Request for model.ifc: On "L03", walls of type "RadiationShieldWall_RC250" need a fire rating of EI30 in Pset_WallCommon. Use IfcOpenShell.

First a look at what the model holds.

```python
import ifcopenshell
import ifcopenshell.util.element

model = ifcopenshell.open("model.ifc")
print(model.schema)
storey = next(s for s in model.by_type("IfcBuildingStorey") if s.Name == "L03")
walls = [e for e in ifcopenshell.util.element.get_decomposition(storey) if e.is_a("IfcWall")]
seen = {}
for e in walls:
    element_type = ifcopenshell.util.element.get_type(e)
    key = (element_type.Name if element_type != e and element_type else None, ifcopenshell.util.element.get_pset(e, "Pset_WallCommon", "FireRating"))
    seen[key] = seen.get(key, 0) + 1
for (name, value), count in sorted(seen.items(), key=str):
    print(count, "x", name, "|", value)
```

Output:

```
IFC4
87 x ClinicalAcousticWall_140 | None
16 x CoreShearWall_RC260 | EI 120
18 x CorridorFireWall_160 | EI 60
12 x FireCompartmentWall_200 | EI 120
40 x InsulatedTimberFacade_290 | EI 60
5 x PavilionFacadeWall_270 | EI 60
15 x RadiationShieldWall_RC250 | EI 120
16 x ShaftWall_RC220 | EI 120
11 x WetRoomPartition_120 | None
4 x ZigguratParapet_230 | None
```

```python
import ifcopenshell
import ifcopenshell.api.pset
import ifcopenshell.util.element

model = ifcopenshell.open("model.ifc")

storey = next(s for s in model.by_type("IfcBuildingStorey") if s.Name == "L03")
walls = [e for e in ifcopenshell.util.element.get_decomposition(storey) if e.is_a("IfcWall")]

count = 0
for e in walls:
    element_type = ifcopenshell.util.element.get_type(e)
    if element_type in (None, e) or element_type.Name != "RadiationShieldWall_RC250":
        continue
    # add_pset returns the element's existing set when there is one.
    pset = ifcopenshell.api.pset.add_pset(model, product=e, name="Pset_WallCommon")
    ifcopenshell.api.pset.edit_pset(model, pset=pset, properties={"FireRating": "EI30"})
    count += 1

print(count, "walls updated")

model.write("model-out.ifc")
```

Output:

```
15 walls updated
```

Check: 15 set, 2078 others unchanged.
